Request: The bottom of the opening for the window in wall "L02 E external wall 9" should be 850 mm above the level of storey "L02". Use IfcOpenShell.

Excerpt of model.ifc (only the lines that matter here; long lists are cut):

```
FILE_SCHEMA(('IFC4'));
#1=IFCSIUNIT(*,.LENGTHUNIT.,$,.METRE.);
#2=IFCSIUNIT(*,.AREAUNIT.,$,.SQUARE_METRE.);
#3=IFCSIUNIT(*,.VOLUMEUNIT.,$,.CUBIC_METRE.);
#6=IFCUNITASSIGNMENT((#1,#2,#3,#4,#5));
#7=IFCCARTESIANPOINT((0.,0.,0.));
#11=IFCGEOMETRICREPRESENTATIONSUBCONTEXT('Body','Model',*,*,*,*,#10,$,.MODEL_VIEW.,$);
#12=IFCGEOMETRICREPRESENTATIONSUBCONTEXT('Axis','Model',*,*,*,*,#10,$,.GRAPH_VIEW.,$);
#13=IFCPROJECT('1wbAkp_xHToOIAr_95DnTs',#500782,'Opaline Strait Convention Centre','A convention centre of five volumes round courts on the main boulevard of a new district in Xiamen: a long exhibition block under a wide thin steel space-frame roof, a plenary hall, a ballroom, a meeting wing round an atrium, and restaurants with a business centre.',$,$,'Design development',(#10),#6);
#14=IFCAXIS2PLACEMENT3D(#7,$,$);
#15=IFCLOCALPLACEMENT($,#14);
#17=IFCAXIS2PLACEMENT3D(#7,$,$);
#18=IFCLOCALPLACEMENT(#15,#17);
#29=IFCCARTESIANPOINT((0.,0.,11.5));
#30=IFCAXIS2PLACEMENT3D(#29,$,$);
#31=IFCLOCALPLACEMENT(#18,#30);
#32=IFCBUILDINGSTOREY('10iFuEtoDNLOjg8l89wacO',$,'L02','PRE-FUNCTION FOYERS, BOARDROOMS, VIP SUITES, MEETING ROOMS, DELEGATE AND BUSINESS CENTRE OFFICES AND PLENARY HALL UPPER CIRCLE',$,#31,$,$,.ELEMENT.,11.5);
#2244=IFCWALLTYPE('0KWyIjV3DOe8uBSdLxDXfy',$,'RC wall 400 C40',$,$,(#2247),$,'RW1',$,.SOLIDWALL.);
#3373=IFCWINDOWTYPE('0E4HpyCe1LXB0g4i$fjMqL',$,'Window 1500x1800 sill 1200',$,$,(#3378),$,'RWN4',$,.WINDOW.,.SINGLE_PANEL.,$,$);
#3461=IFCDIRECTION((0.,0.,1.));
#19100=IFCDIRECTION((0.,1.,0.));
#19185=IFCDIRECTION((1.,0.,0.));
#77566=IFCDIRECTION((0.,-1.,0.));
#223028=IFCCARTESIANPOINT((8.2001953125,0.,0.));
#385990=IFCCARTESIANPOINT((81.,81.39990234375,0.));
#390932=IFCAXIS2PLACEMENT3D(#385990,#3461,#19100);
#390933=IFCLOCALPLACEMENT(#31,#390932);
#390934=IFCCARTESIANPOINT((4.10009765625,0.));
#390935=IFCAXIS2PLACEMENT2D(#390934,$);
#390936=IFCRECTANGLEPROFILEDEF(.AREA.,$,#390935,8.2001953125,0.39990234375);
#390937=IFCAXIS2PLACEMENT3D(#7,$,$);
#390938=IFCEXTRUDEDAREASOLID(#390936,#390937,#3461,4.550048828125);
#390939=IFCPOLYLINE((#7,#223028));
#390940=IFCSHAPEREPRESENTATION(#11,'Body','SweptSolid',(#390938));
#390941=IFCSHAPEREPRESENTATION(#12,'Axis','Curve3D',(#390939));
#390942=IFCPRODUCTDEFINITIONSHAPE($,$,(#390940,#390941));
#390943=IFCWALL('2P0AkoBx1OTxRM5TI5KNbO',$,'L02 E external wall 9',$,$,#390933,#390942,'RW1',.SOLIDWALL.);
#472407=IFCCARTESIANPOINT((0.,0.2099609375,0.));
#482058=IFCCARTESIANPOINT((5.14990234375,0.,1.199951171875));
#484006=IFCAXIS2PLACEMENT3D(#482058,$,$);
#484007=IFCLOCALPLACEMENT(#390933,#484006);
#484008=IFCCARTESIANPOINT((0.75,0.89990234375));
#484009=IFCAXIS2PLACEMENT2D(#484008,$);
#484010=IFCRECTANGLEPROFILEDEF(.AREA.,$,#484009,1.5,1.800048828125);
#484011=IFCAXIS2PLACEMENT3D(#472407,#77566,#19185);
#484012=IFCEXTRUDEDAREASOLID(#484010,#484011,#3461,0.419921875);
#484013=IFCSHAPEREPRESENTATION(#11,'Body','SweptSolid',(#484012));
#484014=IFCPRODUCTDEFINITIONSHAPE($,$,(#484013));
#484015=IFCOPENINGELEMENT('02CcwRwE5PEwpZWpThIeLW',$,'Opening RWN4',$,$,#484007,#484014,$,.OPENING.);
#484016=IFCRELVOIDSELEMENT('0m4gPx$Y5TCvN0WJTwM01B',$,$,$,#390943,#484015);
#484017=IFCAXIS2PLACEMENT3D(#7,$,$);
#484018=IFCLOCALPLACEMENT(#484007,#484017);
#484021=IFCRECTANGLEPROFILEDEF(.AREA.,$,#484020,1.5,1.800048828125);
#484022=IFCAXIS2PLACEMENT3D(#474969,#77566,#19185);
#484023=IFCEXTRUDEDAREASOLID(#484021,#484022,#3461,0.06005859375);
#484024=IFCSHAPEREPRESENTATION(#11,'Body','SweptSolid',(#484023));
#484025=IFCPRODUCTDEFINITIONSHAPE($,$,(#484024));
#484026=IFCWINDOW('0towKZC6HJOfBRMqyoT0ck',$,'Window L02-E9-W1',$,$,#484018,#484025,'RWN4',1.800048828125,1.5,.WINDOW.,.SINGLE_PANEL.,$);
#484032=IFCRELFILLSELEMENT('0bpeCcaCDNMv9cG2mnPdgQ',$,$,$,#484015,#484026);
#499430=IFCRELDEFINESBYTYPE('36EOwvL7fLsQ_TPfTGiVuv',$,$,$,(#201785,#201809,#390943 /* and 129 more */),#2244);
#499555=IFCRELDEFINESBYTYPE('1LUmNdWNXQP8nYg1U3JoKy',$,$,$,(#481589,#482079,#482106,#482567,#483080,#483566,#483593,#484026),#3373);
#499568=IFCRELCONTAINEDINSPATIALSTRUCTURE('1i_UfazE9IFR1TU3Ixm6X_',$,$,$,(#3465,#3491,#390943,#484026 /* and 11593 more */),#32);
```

```python
import numpy as np
import ifcopenshell
import ifcopenshell.api.geometry
import ifcopenshell.geom
import ifcopenshell.util.element
import ifcopenshell.util.placement
import ifcopenshell.util.shape
import ifcopenshell.util.unit

model = ifcopenshell.open("model.ifc")
unit_scale = ifcopenshell.util.unit.calculate_unit_scale(model)

window = model.by_id(484026)
opening = window.FillsVoids[0].RelatingOpeningElement
storey = ifcopenshell.util.element.get_container(window, ifc_class="IfcBuildingStorey")
level = ifcopenshell.util.placement.get_local_placement(storey.ObjectPlacement)[2, 3]

# The opening's origin need not be at the sill, so measure its lowest point.
shape = ifcopenshell.geom.create_shape(ifcopenshell.geom.settings(), opening)
bottom = ifcopenshell.util.shape.get_shape_bottom_elevation(shape, shape.geometry) / unit_scale
dz = level + 0.85 - bottom

shift = np.array([0.0, 0.0, dz])
# The window is placed relative to its opening, so it follows when the opening moves.
matrix = ifcopenshell.util.placement.get_local_placement(opening.ObjectPlacement)
matrix[:3, 3] += shift
ifcopenshell.api.geometry.edit_object_placement(
    model, product=opening, matrix=matrix, is_si=False, should_transform_children=True
)

print(f"moved by {dz * unit_scale:+.3f} m")

model.write("model_edited.ifc")
```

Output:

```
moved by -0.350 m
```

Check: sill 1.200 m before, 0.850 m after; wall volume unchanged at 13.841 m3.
